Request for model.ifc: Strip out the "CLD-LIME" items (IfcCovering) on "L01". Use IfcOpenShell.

First a look at what the model holds.

```python
import ifcopenshell
import ifcopenshell.util.element

model = ifcopenshell.open("model.ifc")
print(model.schema)
storey = next(s for s in model.by_type("IfcBuildingStorey") if s.Name == "L01")
coverings = [e for e in ifcopenshell.util.element.get_decomposition(storey) if e.is_a("IfcCovering")]
seen = {}
for e in coverings:
    element_type = ifcopenshell.util.element.get_type(e)
    name = element_type.Name if element_type not in (None, e) else None
    seen[name] = seen.get(name, 0) + 1
for name, count in sorted(seen.items(), key=str):
    print(count, "x", name)
```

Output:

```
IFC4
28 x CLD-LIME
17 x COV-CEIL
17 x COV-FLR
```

```python
import ifcopenshell
import ifcopenshell.api.root
import ifcopenshell.util.element

model = ifcopenshell.open("model.ifc")

storey = next(s for s in model.by_type("IfcBuildingStorey") if s.Name == "L01")
coverings = [e for e in ifcopenshell.util.element.get_decomposition(storey) if e.is_a("IfcCovering")]
targets = [e for e in coverings if (t := ifcopenshell.util.element.get_type(e)) not in (None, e) and t.Name == "CLD-LIME"]

for e in targets:
    ifcopenshell.api.root.remove_product(model, product=e)
print(len(targets), "removed")

model.write("model-out.ifc")
```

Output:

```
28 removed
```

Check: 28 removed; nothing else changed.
